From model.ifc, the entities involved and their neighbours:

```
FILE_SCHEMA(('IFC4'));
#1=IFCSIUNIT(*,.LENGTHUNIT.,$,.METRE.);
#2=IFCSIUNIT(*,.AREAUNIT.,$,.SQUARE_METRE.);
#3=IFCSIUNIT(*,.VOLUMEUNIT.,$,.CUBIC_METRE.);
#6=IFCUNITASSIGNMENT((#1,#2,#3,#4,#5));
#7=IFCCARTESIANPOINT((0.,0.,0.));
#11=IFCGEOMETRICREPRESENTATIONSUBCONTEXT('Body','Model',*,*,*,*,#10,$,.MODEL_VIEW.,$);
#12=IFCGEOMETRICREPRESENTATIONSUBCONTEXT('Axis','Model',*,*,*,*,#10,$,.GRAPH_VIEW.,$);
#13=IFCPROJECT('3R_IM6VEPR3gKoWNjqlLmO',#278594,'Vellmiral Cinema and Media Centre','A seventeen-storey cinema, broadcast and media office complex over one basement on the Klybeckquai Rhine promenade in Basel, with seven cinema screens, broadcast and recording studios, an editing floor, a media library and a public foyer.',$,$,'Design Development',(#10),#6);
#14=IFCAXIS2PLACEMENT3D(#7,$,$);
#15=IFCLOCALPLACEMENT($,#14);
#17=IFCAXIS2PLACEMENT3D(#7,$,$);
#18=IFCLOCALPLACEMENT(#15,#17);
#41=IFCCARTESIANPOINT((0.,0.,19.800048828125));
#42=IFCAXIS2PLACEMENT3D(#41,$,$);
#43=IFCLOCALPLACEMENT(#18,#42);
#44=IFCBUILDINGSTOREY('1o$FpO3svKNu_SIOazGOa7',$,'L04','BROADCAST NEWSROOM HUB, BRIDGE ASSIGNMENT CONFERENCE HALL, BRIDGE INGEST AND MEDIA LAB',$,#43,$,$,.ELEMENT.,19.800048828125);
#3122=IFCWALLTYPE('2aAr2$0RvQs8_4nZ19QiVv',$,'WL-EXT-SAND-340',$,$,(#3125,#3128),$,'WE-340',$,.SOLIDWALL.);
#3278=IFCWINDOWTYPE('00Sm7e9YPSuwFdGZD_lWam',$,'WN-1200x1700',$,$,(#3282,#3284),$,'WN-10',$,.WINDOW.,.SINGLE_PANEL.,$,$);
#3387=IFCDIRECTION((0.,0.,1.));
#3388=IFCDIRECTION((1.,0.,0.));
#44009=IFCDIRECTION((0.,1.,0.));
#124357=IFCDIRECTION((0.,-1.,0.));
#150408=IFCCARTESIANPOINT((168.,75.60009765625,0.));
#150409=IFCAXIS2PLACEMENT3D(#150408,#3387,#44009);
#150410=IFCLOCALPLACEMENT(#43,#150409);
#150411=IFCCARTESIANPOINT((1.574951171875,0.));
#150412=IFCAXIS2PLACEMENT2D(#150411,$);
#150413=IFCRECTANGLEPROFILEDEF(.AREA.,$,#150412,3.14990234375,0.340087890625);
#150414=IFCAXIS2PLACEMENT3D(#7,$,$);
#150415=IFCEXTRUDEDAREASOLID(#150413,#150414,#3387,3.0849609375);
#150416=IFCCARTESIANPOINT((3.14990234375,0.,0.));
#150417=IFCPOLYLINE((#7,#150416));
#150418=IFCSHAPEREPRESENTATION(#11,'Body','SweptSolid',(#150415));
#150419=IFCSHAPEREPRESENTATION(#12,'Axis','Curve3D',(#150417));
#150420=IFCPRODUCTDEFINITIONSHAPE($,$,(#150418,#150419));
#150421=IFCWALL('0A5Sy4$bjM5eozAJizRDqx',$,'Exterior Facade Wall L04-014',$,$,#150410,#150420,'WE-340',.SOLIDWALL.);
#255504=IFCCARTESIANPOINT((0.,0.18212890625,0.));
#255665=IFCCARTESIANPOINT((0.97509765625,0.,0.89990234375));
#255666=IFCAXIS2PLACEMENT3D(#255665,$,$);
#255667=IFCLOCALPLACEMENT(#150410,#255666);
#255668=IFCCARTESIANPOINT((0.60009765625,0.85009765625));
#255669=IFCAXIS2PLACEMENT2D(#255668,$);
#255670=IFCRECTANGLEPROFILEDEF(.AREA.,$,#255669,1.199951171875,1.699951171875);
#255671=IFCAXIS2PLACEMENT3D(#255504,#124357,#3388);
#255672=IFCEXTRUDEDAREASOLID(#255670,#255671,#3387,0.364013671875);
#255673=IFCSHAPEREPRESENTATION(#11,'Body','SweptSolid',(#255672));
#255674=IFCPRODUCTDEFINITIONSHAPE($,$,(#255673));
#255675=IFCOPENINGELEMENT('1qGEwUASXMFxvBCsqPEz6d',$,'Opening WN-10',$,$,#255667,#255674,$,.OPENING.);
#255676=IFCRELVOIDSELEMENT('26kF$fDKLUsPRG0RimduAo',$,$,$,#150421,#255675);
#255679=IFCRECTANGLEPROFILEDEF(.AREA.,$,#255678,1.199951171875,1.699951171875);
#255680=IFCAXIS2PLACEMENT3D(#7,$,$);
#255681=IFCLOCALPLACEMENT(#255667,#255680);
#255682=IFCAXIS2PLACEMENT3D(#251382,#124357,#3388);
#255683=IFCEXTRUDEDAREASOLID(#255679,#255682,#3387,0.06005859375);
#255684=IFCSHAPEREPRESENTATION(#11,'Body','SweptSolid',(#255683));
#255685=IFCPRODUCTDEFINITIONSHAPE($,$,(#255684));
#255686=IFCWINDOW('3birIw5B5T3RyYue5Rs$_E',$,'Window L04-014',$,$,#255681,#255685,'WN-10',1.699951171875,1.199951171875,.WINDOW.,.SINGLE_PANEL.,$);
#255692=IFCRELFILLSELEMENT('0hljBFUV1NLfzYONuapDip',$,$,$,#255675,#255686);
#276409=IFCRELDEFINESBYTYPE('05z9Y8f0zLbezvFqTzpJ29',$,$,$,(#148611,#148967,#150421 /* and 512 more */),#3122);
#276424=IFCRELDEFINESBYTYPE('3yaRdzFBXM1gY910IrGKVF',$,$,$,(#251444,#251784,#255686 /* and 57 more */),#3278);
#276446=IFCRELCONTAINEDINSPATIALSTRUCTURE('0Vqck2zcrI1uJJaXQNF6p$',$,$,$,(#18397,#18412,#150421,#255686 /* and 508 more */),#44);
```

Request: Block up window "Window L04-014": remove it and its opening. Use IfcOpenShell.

```python
import ifcopenshell
import ifcopenshell.api.feature
import ifcopenshell.api.root
import ifcopenshell.geom
import ifcopenshell.util.shape

model = ifcopenshell.open("model.ifc")
settings = ifcopenshell.geom.settings()


def volume(element):
    """Net volume in cubic metres, openings subtracted."""
    shape = ifcopenshell.geom.create_shape(settings, element)
    return ifcopenshell.util.shape.get_volume(shape.geometry)


window = model.by_id(255686)
opening = window.FillsVoids[0].RelatingOpeningElement
wall = opening.VoidsElements[0].RelatingBuildingElement
before = volume(wall)

ifcopenshell.api.root.remove_product(model, product=window)
ifcopenshell.api.feature.remove_feature(model, feature=opening)

after = volume(wall)

print(f"wall volume {before:.3f} -> {after:.3f} m3")

model.write("model_edited.ifc")
```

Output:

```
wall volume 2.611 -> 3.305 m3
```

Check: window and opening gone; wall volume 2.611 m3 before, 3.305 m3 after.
